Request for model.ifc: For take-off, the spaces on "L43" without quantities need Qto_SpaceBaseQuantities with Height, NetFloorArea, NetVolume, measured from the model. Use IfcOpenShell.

First a look at what the model holds.

```python
import ifcopenshell
import ifcopenshell.util.element
import ifcopenshell.util.unit

model = ifcopenshell.open("model.ifc")
print(model.schema)
for unit_type in ("LENGTHUNIT", "AREAUNIT", "VOLUMEUNIT"):
    print(unit_type, ifcopenshell.util.unit.calculate_unit_scale(model, unit_type))
storey = next(s for s in model.by_type("IfcBuildingStorey") if s.Name == "L43")
spaces = [e for e in ifcopenshell.util.element.get_decomposition(storey) if e.is_a("IfcSpace")]
for e in sorted(spaces, key=lambda e: e.id()):
    print(e.id(), e.is_a(), e.Name, list(ifcopenshell.util.element.get_psets(e, qtos_only=True)), sep=" | ")
```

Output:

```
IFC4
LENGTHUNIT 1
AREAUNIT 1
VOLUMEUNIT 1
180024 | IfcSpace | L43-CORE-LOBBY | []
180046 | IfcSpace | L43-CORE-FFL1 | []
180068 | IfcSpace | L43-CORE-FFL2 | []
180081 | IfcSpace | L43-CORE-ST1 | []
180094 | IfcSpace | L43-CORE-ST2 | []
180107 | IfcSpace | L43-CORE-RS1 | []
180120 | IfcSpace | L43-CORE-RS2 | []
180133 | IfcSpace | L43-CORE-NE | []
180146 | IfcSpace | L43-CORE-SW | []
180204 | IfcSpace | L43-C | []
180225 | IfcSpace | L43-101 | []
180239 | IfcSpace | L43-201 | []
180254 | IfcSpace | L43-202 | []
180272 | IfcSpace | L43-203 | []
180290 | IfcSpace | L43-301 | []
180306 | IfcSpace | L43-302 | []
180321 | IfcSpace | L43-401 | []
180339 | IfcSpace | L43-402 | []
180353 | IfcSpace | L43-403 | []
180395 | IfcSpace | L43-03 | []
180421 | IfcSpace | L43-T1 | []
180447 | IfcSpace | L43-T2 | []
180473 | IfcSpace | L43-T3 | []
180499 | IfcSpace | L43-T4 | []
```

```python
import ifcopenshell
import ifcopenshell.api.pset
import ifcopenshell.geom
import ifcopenshell.util.element
import ifcopenshell.util.shape
import ifcopenshell.util.unit

model = ifcopenshell.open("model.ifc")
unit_scale = ifcopenshell.util.unit.calculate_unit_scale(model)
area_scale = ifcopenshell.util.unit.calculate_unit_scale(model, "AREAUNIT")
volume_scale = ifcopenshell.util.unit.calculate_unit_scale(model, "VOLUMEUNIT")
settings = ifcopenshell.geom.settings()

storey = next(s for s in model.by_type("IfcBuildingStorey") if s.Name == "L43")
spaces = [e for e in ifcopenshell.util.element.get_decomposition(storey) if e.is_a("IfcSpace")]

for e in sorted(spaces, key=lambda e: e.id()):
    if ifcopenshell.util.element.get_psets(e, qtos_only=True, should_inherit=False):
        continue
    # Geometry comes back in metres, in the element's own axes.
    shape = ifcopenshell.geom.create_shape(settings, e)
    values = {
        "Height": ifcopenshell.util.shape.get_z(shape.geometry) / unit_scale,
        "NetFloorArea": ifcopenshell.util.shape.get_footprint_area(shape.geometry) / area_scale,
        "NetVolume": ifcopenshell.util.shape.get_volume(shape.geometry) / volume_scale,
    }
    qto = ifcopenshell.api.pset.add_qto(model, product=e, name="Qto_SpaceBaseQuantities")
    ifcopenshell.api.pset.edit_qto(model, qto=qto, properties=values)
    print(e.id(), {k: round(v, 3) for k, v in values.items()})

model.write("model_edited.ifc")
```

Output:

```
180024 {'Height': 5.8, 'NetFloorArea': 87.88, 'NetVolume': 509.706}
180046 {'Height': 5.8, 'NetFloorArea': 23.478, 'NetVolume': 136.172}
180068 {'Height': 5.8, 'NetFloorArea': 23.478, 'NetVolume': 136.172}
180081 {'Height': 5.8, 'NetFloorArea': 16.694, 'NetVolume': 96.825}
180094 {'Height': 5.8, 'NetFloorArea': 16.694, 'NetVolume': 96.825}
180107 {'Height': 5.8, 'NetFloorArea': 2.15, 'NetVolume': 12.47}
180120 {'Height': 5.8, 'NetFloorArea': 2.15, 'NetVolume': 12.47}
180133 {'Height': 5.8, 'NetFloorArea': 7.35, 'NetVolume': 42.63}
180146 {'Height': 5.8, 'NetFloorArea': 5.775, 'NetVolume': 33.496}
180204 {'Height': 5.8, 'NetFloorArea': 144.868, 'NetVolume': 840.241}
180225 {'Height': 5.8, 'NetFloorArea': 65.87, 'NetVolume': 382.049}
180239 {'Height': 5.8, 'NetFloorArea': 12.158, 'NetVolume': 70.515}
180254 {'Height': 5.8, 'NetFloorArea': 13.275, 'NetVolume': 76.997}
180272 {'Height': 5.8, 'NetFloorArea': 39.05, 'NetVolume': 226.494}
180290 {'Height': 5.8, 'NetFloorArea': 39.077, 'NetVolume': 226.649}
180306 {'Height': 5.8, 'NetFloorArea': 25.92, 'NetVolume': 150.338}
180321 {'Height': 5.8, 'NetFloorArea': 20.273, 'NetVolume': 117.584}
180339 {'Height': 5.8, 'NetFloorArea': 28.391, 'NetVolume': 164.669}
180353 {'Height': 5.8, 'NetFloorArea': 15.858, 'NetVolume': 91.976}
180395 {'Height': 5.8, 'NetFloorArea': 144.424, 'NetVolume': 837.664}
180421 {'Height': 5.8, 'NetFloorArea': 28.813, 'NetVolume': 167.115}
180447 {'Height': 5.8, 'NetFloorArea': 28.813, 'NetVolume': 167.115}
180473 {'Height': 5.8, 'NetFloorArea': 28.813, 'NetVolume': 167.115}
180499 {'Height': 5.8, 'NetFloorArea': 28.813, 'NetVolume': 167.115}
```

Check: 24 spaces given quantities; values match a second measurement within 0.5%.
